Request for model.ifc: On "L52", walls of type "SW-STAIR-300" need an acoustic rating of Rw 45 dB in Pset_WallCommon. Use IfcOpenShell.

First a look at what the model holds.

```python
import ifcopenshell
import ifcopenshell.util.element

model = ifcopenshell.open("model.ifc")
print(model.schema)
storey = next(s for s in model.by_type("IfcBuildingStorey") if s.Name == "L52")
walls = [e for e in ifcopenshell.util.element.get_decomposition(storey) if e.is_a("IfcWall")]
seen = {}
for e in walls:
    element_type = ifcopenshell.util.element.get_type(e)
    key = (element_type.Name if element_type != e and element_type else None, ifcopenshell.util.element.get_pset(e, "Pset_WallCommon", "AcousticRating"))
    seen[key] = seen.get(key, 0) + 1
for (name, value), count in sorted(seen.items(), key=str):
    print(count, "x", name, "|", value)
```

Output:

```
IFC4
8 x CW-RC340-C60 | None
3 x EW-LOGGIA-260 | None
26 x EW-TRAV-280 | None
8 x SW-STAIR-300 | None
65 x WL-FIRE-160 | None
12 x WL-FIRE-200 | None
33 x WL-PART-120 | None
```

```python
import ifcopenshell
import ifcopenshell.api.pset
import ifcopenshell.util.element

model = ifcopenshell.open("model.ifc")

storey = next(s for s in model.by_type("IfcBuildingStorey") if s.Name == "L52")
walls = [e for e in ifcopenshell.util.element.get_decomposition(storey) if e.is_a("IfcWall")]

count = 0
for e in walls:
    element_type = ifcopenshell.util.element.get_type(e)
    if element_type in (None, e) or element_type.Name != "SW-STAIR-300":
        continue
    # add_pset returns the element's existing set when there is one.
    pset = ifcopenshell.api.pset.add_pset(model, product=e, name="Pset_WallCommon")
    ifcopenshell.api.pset.edit_pset(model, pset=pset, properties={"AcousticRating": "Rw 45 dB"})
    count += 1

print(count, "walls updated")

model.write("model_rev.ifc")
```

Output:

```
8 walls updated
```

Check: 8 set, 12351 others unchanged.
